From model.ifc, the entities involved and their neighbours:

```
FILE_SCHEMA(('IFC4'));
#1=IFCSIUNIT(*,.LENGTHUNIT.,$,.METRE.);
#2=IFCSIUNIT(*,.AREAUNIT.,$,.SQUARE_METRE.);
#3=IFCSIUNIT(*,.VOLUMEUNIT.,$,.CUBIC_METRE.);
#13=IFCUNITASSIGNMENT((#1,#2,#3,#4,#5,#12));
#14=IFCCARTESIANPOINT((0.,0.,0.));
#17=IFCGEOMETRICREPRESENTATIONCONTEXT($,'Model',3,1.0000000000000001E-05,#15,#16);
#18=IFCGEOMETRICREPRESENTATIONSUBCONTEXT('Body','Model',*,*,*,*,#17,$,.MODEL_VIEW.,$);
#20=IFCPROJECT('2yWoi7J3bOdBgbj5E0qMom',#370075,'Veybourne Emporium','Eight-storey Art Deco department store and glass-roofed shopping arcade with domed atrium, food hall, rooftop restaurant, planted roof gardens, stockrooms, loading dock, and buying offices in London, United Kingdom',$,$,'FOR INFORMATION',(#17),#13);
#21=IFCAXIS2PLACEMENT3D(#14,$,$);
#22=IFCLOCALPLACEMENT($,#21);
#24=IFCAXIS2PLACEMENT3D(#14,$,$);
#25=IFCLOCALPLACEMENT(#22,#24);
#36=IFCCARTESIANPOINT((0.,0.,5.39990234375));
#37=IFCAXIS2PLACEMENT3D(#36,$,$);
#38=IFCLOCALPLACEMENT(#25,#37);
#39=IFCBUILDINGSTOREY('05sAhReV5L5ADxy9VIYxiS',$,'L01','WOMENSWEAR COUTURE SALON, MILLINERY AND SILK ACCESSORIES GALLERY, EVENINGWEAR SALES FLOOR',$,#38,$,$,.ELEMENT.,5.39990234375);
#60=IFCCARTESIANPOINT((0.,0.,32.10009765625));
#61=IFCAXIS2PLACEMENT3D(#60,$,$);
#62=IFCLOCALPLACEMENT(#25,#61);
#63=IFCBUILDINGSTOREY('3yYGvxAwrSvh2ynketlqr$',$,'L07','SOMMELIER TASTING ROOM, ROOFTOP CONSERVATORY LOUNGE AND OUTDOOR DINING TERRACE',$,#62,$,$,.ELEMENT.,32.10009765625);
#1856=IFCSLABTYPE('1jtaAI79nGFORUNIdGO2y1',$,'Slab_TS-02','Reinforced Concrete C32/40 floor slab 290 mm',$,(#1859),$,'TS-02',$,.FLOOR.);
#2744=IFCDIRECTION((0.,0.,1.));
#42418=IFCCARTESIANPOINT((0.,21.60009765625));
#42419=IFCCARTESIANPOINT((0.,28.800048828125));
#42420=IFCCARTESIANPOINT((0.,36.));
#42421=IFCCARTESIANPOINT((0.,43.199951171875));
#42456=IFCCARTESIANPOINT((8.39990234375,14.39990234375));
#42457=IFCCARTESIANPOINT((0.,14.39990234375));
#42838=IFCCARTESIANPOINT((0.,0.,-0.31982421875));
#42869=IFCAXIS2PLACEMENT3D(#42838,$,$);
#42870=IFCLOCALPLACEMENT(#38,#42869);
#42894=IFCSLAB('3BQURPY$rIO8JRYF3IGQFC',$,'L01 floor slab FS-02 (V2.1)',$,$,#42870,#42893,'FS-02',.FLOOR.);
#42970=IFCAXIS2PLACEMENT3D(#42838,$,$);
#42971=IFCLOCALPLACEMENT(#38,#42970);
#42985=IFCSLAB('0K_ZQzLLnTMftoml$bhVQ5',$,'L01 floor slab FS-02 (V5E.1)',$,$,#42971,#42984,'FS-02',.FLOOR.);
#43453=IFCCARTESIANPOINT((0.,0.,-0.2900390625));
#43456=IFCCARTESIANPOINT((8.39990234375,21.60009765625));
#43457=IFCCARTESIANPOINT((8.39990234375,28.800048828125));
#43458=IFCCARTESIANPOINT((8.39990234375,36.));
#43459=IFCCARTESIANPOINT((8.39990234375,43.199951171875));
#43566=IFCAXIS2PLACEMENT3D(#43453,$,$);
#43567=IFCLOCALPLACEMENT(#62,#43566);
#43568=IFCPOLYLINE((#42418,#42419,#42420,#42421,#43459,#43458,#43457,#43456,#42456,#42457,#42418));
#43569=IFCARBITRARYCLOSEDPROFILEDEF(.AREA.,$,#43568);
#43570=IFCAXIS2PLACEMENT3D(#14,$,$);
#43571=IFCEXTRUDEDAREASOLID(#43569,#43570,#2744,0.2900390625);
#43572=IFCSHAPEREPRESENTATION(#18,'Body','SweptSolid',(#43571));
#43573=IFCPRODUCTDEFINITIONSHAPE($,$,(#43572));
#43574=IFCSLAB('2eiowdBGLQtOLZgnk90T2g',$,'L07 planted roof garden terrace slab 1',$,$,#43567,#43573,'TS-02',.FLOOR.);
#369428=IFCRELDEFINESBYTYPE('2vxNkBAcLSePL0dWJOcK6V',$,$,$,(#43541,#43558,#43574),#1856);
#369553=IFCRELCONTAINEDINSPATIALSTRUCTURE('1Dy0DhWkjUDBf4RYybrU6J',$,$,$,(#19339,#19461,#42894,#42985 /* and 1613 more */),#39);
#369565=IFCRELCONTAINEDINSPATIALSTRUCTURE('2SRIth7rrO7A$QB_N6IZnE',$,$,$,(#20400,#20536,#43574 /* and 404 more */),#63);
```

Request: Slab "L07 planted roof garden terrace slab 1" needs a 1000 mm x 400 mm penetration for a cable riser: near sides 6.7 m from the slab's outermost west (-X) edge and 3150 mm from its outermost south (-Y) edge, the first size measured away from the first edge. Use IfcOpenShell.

```python
import numpy as np
import ifcopenshell
import ifcopenshell.api.feature
import ifcopenshell.api.geometry
import ifcopenshell.api.root
import ifcopenshell.geom
import ifcopenshell.util.placement
import ifcopenshell.util.representation
import ifcopenshell.util.shape
import ifcopenshell.util.unit

model = ifcopenshell.open("model.ifc")
unit_scale = ifcopenshell.util.unit.calculate_unit_scale(model)
settings = ifcopenshell.geom.settings()


def volume(element):
    """Net volume in cubic metres, openings subtracted."""
    shape = ifcopenshell.geom.create_shape(settings, element)
    return ifcopenshell.util.shape.get_volume(shape.geometry)


slab = model.by_guid("2eiowdBGLQtOLZgnk90T2g")
before = volume(slab)

# Extent in the slab's own axes, in metres. The edges named are its -X and -Y sides.
slab_shape = ifcopenshell.geom.create_shape(settings, slab)
vertices = ifcopenshell.util.shape.get_vertices(slab_shape.geometry)
x_min, y_min, bottom = vertices.min(axis=0)
top = vertices[:, 2].max()

opening = ifcopenshell.api.root.create_entity(model, ifc_class="IfcOpeningElement", name="Cable riser opening", predefined_type="OPENING")
context = ifcopenshell.util.representation.get_context(model, "Model", "Body", "MODEL_VIEW")
width, depth = 1, 0.4
outline = [(0.0, 0.0), (width, 0.0), (width, depth), (0.0, depth), (0.0, 0.0)]
# Overshoot both faces by 50 mm so the cut is clean.
shape = ifcopenshell.api.geometry.add_slab_representation(
    model, context=context, depth=top - bottom + 0.1, polyline=outline
)
ifcopenshell.api.geometry.assign_representation(model, product=opening, representation=shape)

matrix = ifcopenshell.util.placement.get_local_placement(slab.ObjectPlacement)
matrix[:, 3] = matrix @ np.append(np.array([x_min + 6.7, y_min + 3.15, bottom - 0.05]) / unit_scale, 1.0)
ifcopenshell.api.geometry.edit_object_placement(model, product=opening, matrix=matrix, is_si=False)
ifcopenshell.api.feature.add_feature(model, feature=opening, element=slab)

after = volume(slab)

print(f"slab volume {before:.3f} -> {after:.3f} m3")

model.write("model_updated.ifc")
```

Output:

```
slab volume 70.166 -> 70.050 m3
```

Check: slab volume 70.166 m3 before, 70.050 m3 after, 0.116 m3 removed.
